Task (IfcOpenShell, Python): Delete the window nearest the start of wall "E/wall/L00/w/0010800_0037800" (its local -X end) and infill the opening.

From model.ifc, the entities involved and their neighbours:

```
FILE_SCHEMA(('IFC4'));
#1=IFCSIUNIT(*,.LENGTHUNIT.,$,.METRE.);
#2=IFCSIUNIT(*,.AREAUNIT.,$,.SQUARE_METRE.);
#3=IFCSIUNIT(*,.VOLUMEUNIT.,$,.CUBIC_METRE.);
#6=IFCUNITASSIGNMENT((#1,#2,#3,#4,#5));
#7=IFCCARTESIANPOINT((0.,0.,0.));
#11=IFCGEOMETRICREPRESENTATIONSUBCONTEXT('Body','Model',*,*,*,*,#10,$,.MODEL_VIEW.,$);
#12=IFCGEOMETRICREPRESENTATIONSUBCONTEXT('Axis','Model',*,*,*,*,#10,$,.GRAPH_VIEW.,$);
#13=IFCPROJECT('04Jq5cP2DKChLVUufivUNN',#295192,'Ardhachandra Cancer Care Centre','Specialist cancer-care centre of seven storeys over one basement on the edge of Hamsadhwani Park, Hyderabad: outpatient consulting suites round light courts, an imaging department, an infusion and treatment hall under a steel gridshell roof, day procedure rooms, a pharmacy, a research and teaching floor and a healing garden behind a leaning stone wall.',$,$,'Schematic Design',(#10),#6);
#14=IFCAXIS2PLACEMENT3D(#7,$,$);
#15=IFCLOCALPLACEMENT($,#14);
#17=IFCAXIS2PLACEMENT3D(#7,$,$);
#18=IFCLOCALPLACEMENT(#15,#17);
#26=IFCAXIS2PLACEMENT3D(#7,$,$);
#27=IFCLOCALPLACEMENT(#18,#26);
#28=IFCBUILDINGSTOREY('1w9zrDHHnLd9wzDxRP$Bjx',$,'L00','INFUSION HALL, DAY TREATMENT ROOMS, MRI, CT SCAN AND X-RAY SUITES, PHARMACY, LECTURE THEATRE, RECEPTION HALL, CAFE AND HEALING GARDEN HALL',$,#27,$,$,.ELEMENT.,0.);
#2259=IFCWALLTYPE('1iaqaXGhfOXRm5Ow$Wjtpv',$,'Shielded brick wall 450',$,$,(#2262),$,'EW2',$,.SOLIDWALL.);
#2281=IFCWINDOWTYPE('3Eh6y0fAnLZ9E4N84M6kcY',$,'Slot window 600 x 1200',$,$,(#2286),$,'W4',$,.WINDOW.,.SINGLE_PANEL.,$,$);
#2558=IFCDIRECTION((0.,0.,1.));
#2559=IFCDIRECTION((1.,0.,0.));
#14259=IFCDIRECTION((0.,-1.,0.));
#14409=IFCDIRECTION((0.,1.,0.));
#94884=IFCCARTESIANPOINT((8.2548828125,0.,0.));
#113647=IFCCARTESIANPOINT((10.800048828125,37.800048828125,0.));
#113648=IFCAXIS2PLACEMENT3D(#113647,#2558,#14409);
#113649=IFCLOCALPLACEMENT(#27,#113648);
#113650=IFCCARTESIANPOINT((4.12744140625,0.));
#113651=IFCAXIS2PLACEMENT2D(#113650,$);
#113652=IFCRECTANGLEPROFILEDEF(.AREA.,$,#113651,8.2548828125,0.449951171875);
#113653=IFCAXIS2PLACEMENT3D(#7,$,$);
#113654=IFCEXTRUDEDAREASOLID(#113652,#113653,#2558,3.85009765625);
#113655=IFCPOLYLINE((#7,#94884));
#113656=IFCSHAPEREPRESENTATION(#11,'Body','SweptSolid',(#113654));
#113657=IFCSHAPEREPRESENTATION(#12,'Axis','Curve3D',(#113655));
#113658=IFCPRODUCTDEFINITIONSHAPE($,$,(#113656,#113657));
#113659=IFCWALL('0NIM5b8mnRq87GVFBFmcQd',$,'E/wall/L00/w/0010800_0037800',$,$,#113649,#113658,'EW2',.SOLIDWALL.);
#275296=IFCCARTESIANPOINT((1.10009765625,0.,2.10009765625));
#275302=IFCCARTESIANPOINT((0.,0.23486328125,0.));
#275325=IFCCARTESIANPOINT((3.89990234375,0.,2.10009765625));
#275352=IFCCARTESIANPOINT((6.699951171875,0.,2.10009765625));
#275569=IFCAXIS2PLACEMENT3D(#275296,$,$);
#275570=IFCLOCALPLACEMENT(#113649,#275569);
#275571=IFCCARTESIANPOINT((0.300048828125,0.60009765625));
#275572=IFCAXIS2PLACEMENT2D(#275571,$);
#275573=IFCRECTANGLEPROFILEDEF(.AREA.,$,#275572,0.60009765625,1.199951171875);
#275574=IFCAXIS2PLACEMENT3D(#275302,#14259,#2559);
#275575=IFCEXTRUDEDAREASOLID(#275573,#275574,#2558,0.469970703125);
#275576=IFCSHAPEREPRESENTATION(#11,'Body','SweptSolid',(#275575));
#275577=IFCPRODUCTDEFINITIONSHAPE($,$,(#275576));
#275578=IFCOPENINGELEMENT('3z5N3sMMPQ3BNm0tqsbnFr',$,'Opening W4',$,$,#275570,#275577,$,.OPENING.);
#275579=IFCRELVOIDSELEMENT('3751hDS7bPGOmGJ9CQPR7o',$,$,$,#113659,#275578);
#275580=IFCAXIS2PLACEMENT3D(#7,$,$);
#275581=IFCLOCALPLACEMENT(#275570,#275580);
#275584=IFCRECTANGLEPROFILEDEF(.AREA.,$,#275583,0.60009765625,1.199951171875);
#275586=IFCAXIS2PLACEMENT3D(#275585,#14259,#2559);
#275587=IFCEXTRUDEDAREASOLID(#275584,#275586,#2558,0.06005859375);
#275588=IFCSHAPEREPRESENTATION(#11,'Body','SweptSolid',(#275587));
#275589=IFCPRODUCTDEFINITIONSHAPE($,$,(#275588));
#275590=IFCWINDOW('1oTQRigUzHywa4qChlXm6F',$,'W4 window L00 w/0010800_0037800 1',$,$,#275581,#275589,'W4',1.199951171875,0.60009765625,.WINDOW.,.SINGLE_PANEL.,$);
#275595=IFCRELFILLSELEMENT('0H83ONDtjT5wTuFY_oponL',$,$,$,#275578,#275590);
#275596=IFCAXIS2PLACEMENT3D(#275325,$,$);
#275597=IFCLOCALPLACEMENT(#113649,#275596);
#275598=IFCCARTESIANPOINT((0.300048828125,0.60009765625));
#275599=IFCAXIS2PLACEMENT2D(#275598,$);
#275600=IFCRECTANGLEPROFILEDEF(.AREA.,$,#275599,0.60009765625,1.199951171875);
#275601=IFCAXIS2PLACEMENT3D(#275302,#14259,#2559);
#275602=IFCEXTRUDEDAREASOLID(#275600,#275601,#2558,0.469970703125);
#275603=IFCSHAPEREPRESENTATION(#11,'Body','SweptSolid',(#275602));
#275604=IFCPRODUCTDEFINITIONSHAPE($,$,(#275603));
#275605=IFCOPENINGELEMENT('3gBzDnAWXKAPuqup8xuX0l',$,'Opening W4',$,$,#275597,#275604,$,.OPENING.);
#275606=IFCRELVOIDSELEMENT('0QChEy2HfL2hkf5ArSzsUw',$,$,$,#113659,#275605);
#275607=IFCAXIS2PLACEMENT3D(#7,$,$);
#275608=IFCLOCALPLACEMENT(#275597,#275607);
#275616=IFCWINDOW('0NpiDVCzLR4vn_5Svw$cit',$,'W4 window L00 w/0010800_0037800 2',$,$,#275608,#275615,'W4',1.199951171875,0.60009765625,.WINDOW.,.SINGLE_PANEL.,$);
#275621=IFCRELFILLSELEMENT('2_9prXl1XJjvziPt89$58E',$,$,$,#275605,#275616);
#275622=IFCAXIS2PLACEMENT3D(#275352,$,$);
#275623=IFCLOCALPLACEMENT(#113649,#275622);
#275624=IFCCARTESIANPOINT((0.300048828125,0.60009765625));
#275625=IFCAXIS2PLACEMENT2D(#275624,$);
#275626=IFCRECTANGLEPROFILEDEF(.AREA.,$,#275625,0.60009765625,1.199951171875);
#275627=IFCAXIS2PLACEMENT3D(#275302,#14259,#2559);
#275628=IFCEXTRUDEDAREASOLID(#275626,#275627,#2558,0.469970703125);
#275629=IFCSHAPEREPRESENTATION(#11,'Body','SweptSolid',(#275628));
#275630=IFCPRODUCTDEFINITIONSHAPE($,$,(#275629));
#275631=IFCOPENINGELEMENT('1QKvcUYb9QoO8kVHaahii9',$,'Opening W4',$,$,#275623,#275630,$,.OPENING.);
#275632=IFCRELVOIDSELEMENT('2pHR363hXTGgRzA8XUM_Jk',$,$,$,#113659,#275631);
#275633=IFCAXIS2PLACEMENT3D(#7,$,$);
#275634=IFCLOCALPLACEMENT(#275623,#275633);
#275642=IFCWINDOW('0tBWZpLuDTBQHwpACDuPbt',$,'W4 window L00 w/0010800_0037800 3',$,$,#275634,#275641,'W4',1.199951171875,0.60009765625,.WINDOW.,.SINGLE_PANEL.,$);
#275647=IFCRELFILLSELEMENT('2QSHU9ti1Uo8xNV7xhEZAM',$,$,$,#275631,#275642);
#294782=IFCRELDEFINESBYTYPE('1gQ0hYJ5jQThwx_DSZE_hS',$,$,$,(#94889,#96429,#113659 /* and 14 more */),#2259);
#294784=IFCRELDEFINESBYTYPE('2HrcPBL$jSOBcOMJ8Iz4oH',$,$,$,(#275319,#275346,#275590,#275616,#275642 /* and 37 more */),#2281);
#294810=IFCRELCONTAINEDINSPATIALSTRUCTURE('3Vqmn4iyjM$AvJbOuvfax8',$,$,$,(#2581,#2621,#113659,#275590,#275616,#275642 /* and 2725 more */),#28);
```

```python
import ifcopenshell
import ifcopenshell.api.feature
import ifcopenshell.api.root
import ifcopenshell.geom
import ifcopenshell.util.shape

model = ifcopenshell.open("model.ifc")
settings = ifcopenshell.geom.settings()


def volume(element):
    """Net volume in cubic metres, openings subtracted."""
    shape = ifcopenshell.geom.create_shape(settings, element)
    return ifcopenshell.util.shape.get_volume(shape.geometry)


window = model.by_id(275590)
opening = window.FillsVoids[0].RelatingOpeningElement
wall = opening.VoidsElements[0].RelatingBuildingElement
before = volume(wall)

ifcopenshell.api.root.remove_product(model, product=window)
ifcopenshell.api.feature.remove_feature(model, feature=opening)

after = volume(wall)

print(f"wall volume {before:.3f} -> {after:.3f} m3")

model.write("model-out.ifc")
```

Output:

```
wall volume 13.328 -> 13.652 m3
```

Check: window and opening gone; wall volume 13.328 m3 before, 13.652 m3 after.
